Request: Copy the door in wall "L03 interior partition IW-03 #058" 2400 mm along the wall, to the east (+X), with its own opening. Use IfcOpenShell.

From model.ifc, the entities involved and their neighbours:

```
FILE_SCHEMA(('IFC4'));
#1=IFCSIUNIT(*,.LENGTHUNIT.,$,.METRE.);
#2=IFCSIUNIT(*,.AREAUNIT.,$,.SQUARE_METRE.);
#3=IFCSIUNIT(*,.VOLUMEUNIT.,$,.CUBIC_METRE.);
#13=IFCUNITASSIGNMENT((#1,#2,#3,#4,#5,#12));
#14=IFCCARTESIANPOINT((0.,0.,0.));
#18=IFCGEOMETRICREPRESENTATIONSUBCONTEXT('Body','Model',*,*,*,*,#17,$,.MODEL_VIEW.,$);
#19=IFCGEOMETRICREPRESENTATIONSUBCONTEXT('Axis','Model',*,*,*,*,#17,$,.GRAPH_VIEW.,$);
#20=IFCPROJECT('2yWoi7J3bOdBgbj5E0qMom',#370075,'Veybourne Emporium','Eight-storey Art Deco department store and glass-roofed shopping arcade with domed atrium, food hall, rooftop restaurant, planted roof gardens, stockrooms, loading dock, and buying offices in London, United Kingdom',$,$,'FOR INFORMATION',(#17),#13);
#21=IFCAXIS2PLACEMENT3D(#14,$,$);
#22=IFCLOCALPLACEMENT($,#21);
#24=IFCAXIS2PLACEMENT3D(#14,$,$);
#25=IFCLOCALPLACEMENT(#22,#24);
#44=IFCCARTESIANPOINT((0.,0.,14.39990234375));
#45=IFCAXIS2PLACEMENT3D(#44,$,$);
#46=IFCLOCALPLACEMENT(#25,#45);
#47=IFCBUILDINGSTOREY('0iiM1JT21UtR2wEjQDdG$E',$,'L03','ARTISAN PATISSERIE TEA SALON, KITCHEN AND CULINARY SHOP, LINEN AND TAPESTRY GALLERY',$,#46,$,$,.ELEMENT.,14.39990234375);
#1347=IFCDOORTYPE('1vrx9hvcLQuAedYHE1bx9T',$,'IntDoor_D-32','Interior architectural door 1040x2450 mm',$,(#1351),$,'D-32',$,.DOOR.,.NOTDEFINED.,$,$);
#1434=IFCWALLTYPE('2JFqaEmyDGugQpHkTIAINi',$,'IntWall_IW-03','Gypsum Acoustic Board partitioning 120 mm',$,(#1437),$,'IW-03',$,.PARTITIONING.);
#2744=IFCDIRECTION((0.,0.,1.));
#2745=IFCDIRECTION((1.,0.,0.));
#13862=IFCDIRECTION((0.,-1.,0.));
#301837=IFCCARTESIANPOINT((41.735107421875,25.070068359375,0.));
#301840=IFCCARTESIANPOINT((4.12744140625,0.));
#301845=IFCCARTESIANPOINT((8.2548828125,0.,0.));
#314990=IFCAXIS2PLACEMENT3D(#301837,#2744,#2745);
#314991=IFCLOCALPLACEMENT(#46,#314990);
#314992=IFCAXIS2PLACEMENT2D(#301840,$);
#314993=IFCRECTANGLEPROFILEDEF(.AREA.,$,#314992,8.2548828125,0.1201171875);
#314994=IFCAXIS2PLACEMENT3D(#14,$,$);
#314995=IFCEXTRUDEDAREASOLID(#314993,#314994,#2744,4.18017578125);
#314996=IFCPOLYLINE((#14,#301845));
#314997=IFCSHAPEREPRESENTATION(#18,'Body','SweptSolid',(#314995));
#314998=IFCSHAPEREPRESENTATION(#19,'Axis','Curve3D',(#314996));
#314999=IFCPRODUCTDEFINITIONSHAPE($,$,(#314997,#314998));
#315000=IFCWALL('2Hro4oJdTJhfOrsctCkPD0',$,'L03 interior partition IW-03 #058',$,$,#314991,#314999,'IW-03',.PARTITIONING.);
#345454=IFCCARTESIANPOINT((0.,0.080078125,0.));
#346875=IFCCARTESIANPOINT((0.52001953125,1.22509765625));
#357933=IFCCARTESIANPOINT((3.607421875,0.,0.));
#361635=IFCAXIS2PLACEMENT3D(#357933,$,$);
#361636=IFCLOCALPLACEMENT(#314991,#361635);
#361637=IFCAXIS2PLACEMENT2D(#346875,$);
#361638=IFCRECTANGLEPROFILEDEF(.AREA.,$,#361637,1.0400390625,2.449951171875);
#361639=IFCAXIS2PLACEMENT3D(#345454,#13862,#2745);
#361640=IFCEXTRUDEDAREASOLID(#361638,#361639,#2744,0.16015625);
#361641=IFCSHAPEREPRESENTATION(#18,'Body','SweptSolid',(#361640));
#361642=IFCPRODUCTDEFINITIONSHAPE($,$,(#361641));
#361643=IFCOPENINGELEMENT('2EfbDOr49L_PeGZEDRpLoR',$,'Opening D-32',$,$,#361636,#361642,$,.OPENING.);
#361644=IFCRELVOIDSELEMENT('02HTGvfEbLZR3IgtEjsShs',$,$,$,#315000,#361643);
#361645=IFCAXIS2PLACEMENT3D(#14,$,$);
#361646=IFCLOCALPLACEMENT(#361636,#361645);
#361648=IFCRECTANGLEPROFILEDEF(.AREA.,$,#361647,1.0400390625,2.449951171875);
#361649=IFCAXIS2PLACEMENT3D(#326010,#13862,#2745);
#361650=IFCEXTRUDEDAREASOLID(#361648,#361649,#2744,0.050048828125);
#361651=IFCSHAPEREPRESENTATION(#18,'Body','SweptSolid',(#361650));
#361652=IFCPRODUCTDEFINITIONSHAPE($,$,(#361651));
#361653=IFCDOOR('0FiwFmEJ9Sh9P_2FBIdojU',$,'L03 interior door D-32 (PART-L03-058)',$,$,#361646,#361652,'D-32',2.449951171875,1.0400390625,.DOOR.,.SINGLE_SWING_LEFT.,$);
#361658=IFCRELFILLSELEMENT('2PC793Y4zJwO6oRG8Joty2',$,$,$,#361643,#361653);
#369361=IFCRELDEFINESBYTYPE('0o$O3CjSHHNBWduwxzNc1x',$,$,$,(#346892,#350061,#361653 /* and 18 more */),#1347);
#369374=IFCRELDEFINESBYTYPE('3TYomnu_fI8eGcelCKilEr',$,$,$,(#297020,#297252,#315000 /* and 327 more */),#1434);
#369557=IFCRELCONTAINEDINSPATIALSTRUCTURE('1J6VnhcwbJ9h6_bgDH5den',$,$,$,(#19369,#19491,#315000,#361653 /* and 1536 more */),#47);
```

```python
import ifcopenshell
import ifcopenshell.api.feature
import ifcopenshell.api.geometry
import ifcopenshell.api.root
import ifcopenshell.geom
import ifcopenshell.util.element
import ifcopenshell.util.placement
import ifcopenshell.util.shape
import ifcopenshell.util.unit

model = ifcopenshell.open("model.ifc")
unit_scale = ifcopenshell.util.unit.calculate_unit_scale(model)
settings = ifcopenshell.geom.settings()


def volume(element):
    """Net volume in cubic metres, openings subtracted."""
    shape = ifcopenshell.geom.create_shape(settings, element)
    return ifcopenshell.util.shape.get_volume(shape.geometry)


door = model.by_guid("0FiwFmEJ9Sh9P_2FBIdojU")
opening = door.FillsVoids[0].RelatingOpeningElement
wall = opening.VoidsElements[0].RelatingBuildingElement
before = volume(wall)
shift = ifcopenshell.util.placement.get_local_placement(wall.ObjectPlacement)[:3, 0] * 2.4 / unit_scale

# copy_class copies the void relationship, type, container and properties, but no geometry.
new_opening = ifcopenshell.api.root.copy_class(model, product=opening)
new_opening.Representation = ifcopenshell.util.element.copy_deep(
    model, opening.Representation, exclude=["IfcGeometricRepresentationContext", "IfcRepresentationMap"]
)
new_door = ifcopenshell.api.root.copy_class(model, product=door)
new_door.Representation = ifcopenshell.util.element.copy_deep(
    model, door.Representation, exclude=["IfcGeometricRepresentationContext", "IfcRepresentationMap"]
)
new_door.Tag = None
ifcopenshell.api.feature.add_filling(model, opening=new_opening, element=new_door)

for old, new in ((opening, new_opening), (door, new_door)):
    matrix = ifcopenshell.util.placement.get_local_placement(old.ObjectPlacement)
    matrix[:3, 3] += shift
    ifcopenshell.api.geometry.edit_object_placement(model, product=new, matrix=matrix, is_si=False)

after = volume(wall)

print(f"wall volume {before:.3f} -> {after:.3f} m3")

model.write("model_v2.ifc")
```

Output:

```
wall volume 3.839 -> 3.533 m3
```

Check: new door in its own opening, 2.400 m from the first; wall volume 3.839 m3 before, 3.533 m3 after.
